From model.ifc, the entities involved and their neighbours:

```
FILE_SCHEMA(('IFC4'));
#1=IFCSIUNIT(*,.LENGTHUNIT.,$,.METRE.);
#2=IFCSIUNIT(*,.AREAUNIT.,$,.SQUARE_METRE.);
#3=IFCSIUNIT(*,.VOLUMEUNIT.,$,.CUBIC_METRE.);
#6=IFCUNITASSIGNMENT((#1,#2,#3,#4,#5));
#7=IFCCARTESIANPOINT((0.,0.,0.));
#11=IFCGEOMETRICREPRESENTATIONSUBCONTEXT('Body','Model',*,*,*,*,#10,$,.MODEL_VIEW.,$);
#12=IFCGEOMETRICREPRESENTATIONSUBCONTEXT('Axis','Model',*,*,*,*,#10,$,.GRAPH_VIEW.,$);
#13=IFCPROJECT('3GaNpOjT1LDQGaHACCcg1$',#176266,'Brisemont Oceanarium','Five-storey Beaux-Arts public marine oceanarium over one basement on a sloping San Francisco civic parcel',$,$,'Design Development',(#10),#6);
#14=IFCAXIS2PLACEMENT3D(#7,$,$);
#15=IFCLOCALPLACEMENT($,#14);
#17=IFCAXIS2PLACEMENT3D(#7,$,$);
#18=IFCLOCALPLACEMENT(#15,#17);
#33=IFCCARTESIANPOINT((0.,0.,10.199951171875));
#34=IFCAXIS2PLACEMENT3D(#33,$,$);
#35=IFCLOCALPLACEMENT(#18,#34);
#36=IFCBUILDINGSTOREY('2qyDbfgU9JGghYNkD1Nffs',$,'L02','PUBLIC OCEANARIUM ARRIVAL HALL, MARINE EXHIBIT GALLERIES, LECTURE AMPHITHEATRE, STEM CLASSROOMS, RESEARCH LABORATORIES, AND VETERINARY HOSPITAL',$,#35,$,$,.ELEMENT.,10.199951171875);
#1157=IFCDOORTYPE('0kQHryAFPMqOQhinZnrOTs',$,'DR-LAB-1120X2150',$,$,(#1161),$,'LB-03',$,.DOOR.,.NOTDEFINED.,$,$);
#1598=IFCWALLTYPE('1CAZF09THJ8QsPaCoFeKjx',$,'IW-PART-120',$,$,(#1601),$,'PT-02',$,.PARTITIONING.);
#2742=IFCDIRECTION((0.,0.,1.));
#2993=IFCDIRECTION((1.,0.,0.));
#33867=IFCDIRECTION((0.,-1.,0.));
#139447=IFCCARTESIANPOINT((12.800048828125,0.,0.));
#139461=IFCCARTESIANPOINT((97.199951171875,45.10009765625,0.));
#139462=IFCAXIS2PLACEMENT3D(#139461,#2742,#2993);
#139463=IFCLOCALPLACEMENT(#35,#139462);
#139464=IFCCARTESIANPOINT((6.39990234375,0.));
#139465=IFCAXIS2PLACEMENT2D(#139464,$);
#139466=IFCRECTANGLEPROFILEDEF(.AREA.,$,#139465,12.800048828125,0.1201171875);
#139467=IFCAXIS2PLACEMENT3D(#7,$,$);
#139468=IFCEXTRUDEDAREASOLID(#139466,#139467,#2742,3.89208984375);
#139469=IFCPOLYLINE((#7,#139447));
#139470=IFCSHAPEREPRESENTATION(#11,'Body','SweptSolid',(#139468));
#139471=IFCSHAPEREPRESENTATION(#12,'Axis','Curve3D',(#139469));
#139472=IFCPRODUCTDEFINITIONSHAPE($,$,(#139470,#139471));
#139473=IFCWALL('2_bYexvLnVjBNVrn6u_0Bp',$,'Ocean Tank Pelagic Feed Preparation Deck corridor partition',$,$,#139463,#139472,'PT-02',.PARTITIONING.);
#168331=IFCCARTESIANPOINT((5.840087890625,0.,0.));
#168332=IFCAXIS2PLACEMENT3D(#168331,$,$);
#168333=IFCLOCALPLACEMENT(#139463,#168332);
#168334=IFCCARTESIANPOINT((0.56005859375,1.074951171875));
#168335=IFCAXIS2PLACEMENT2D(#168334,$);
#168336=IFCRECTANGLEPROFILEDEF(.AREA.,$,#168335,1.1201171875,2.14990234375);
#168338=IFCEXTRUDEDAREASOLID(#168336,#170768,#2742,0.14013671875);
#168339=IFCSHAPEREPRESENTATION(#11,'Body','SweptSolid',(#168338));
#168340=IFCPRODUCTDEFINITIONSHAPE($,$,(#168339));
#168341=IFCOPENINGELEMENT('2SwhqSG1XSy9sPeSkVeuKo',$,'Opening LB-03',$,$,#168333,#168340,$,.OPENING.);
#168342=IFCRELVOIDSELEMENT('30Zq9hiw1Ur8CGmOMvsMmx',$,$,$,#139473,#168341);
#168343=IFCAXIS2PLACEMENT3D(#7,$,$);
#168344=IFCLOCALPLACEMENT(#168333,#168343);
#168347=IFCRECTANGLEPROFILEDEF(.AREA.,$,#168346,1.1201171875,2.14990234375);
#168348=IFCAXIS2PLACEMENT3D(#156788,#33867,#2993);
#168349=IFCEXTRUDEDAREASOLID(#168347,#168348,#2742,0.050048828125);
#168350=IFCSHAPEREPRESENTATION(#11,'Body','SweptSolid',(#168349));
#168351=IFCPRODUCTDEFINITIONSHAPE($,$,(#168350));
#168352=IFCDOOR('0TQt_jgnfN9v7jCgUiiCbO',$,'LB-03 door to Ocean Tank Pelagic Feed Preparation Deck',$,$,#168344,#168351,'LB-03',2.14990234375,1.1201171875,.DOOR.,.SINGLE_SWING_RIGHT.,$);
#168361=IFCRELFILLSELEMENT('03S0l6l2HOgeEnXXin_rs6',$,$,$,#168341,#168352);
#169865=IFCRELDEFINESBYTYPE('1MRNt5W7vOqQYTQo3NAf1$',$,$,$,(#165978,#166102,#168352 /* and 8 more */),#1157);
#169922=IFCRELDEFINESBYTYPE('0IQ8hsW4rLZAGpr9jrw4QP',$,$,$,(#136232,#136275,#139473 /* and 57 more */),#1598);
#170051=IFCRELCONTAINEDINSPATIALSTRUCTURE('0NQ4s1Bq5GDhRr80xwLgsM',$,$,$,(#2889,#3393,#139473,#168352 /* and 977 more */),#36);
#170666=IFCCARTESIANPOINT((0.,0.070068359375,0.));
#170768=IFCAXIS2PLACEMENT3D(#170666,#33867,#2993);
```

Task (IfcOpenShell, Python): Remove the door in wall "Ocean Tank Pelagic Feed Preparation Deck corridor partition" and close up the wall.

```python
import ifcopenshell
import ifcopenshell.api.feature
import ifcopenshell.api.root
import ifcopenshell.geom
import ifcopenshell.util.shape

model = ifcopenshell.open("model.ifc")
settings = ifcopenshell.geom.settings()


def volume(element):
    """Net volume in cubic metres, openings subtracted."""
    shape = ifcopenshell.geom.create_shape(settings, element)
    return ifcopenshell.util.shape.get_volume(shape.geometry)


door = model.by_id(168352)
opening = door.FillsVoids[0].RelatingOpeningElement
wall = opening.VoidsElements[0].RelatingBuildingElement
before = volume(wall)

ifcopenshell.api.root.remove_product(model, product=door)
ifcopenshell.api.feature.remove_feature(model, feature=opening)

after = volume(wall)

print(f"wall volume {before:.3f} -> {after:.3f} m3")

model.write("model_rev.ifc")
```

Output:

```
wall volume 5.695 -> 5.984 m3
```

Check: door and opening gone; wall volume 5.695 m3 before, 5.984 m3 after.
